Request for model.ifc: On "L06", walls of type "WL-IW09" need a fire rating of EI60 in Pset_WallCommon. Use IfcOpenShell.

First a look at what the model holds.

```python
import ifcopenshell
import ifcopenshell.util.element

model = ifcopenshell.open("model.ifc")
print(model.schema)
storey = next(s for s in model.by_type("IfcBuildingStorey") if s.Name == "L06")
walls = [e for e in ifcopenshell.util.element.get_decomposition(storey) if e.is_a("IfcWall")]
seen = {}
for e in walls:
    element_type = ifcopenshell.util.element.get_type(e)
    key = (element_type.Name if element_type != e and element_type else None, ifcopenshell.util.element.get_pset(e, "Pset_WallCommon", "FireRating"))
    seen[key] = seen.get(key, 0) + 1
for (name, value), count in sorted(seen.items(), key=str):
    print(count, "x", name, "|", value)
```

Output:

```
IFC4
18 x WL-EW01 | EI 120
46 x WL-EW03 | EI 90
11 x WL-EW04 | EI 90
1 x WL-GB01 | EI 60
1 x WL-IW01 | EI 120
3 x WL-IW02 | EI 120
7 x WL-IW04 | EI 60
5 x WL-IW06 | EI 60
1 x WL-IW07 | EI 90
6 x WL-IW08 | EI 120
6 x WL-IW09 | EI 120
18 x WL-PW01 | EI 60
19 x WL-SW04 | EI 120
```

```python
import ifcopenshell
import ifcopenshell.api.pset
import ifcopenshell.util.element

model = ifcopenshell.open("model.ifc")

storey = next(s for s in model.by_type("IfcBuildingStorey") if s.Name == "L06")
walls = [e for e in ifcopenshell.util.element.get_decomposition(storey) if e.is_a("IfcWall")]

count = 0
for e in walls:
    element_type = ifcopenshell.util.element.get_type(e)
    if element_type in (None, e) or element_type.Name != "WL-IW09":
        continue
    # add_pset returns the element's existing set when there is one.
    pset = ifcopenshell.api.pset.add_pset(model, product=e, name="Pset_WallCommon")
    ifcopenshell.api.pset.edit_pset(model, pset=pset, properties={"FireRating": "EI60"})
    count += 1

print(count, "walls updated")

model.write("model_edited.ifc")
```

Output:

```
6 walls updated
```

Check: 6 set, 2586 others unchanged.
